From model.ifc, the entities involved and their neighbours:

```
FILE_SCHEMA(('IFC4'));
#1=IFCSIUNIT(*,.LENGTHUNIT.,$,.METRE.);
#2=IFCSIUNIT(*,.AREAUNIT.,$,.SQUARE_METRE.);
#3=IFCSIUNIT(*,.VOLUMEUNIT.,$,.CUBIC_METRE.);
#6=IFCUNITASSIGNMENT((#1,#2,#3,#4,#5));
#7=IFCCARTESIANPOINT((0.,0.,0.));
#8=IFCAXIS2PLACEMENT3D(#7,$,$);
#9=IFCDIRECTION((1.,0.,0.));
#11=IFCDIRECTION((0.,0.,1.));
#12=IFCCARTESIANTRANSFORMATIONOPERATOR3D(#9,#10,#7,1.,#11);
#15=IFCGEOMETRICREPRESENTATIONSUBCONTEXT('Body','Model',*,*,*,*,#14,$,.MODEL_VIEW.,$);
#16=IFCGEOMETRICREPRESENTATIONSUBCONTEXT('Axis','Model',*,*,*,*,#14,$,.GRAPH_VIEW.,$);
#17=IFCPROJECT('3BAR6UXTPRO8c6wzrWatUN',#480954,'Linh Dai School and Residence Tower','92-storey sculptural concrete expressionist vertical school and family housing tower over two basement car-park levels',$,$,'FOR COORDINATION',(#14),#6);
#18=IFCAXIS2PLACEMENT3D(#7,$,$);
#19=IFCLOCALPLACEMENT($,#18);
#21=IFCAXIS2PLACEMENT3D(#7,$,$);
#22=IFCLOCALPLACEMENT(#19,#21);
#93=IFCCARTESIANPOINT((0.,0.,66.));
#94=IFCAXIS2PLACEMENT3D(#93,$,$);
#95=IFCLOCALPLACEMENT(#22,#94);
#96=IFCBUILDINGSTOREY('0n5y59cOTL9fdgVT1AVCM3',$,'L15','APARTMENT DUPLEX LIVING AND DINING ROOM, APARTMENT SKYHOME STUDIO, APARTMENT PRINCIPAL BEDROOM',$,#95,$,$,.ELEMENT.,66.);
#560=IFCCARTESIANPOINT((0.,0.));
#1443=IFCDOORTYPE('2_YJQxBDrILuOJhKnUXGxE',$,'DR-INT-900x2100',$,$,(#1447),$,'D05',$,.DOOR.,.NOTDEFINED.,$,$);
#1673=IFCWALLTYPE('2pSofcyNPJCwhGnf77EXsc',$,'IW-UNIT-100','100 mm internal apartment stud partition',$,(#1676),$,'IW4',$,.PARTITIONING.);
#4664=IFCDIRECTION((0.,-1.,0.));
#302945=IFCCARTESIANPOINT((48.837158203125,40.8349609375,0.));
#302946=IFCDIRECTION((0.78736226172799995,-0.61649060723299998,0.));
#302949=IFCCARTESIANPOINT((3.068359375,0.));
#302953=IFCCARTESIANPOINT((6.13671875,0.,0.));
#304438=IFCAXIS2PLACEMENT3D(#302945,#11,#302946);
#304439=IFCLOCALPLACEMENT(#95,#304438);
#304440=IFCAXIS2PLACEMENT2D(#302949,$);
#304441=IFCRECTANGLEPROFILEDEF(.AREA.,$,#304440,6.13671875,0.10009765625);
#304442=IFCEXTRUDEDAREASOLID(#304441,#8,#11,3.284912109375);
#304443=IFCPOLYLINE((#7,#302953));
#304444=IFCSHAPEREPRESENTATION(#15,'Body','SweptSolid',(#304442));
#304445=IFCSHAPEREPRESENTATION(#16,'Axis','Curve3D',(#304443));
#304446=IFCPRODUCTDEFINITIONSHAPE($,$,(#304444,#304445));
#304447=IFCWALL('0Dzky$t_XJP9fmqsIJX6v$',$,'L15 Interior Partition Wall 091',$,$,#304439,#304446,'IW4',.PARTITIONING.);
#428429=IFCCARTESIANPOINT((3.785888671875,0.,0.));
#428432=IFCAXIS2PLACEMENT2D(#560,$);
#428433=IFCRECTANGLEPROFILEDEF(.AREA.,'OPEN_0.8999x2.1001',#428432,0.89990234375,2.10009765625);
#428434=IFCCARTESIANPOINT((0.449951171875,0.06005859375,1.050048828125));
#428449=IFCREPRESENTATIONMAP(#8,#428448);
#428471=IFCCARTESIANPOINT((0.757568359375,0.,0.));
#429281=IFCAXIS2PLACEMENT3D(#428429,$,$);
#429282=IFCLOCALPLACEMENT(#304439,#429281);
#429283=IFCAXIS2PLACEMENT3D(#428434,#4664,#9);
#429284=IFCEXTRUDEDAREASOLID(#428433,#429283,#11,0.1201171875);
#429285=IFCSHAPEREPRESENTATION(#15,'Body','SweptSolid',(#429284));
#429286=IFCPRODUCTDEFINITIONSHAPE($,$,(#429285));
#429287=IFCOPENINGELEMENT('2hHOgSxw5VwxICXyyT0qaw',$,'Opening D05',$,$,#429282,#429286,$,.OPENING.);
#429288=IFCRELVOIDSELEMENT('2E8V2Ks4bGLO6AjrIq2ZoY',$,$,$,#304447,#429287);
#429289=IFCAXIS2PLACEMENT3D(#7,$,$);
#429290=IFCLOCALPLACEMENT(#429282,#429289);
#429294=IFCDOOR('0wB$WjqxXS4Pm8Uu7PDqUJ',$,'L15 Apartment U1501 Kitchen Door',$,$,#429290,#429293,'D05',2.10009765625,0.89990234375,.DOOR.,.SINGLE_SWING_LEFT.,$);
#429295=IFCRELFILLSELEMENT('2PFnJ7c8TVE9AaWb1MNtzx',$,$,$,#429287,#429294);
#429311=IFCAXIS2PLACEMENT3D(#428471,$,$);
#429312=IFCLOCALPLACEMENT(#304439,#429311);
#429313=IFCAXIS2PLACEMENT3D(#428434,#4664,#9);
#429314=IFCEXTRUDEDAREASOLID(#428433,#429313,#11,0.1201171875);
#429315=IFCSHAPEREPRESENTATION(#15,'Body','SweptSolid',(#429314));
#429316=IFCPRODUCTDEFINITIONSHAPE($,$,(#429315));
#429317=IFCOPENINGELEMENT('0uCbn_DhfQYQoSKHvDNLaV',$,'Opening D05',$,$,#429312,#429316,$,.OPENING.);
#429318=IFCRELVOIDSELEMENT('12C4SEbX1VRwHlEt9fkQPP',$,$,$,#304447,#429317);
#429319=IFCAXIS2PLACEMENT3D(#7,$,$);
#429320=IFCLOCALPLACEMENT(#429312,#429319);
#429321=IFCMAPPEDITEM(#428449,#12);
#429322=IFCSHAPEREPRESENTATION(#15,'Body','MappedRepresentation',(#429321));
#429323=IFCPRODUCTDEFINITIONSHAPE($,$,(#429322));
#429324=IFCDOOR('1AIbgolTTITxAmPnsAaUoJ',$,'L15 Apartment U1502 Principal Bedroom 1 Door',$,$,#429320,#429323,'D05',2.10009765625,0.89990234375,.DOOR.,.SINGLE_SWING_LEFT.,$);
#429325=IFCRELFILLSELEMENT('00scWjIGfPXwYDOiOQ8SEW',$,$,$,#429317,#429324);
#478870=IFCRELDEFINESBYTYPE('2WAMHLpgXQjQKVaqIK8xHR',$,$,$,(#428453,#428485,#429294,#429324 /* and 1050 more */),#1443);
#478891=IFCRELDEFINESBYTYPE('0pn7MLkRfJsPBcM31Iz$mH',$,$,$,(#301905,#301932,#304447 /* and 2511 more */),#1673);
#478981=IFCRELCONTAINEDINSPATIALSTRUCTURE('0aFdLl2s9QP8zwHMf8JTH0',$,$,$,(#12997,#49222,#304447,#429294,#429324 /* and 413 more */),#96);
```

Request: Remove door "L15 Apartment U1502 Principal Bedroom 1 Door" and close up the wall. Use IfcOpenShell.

```python
import ifcopenshell
import ifcopenshell.api.feature
import ifcopenshell.api.root
import ifcopenshell.geom
import ifcopenshell.util.shape

model = ifcopenshell.open("model.ifc")
settings = ifcopenshell.geom.settings()


def volume(element):
    """Net volume in cubic metres, openings subtracted."""
    shape = ifcopenshell.geom.create_shape(settings, element)
    return ifcopenshell.util.shape.get_volume(shape.geometry)


door = model.by_guid("1AIbgolTTITxAmPnsAaUoJ")
opening = door.FillsVoids[0].RelatingOpeningElement
wall = opening.VoidsElements[0].RelatingBuildingElement
before = volume(wall)

ifcopenshell.api.root.remove_product(model, product=door)
ifcopenshell.api.feature.remove_feature(model, feature=opening)

after = volume(wall)

print(f"wall volume {before:.3f} -> {after:.3f} m3")

model.write("model_rev.ifc")
```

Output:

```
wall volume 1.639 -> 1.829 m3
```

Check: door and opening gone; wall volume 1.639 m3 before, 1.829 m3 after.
